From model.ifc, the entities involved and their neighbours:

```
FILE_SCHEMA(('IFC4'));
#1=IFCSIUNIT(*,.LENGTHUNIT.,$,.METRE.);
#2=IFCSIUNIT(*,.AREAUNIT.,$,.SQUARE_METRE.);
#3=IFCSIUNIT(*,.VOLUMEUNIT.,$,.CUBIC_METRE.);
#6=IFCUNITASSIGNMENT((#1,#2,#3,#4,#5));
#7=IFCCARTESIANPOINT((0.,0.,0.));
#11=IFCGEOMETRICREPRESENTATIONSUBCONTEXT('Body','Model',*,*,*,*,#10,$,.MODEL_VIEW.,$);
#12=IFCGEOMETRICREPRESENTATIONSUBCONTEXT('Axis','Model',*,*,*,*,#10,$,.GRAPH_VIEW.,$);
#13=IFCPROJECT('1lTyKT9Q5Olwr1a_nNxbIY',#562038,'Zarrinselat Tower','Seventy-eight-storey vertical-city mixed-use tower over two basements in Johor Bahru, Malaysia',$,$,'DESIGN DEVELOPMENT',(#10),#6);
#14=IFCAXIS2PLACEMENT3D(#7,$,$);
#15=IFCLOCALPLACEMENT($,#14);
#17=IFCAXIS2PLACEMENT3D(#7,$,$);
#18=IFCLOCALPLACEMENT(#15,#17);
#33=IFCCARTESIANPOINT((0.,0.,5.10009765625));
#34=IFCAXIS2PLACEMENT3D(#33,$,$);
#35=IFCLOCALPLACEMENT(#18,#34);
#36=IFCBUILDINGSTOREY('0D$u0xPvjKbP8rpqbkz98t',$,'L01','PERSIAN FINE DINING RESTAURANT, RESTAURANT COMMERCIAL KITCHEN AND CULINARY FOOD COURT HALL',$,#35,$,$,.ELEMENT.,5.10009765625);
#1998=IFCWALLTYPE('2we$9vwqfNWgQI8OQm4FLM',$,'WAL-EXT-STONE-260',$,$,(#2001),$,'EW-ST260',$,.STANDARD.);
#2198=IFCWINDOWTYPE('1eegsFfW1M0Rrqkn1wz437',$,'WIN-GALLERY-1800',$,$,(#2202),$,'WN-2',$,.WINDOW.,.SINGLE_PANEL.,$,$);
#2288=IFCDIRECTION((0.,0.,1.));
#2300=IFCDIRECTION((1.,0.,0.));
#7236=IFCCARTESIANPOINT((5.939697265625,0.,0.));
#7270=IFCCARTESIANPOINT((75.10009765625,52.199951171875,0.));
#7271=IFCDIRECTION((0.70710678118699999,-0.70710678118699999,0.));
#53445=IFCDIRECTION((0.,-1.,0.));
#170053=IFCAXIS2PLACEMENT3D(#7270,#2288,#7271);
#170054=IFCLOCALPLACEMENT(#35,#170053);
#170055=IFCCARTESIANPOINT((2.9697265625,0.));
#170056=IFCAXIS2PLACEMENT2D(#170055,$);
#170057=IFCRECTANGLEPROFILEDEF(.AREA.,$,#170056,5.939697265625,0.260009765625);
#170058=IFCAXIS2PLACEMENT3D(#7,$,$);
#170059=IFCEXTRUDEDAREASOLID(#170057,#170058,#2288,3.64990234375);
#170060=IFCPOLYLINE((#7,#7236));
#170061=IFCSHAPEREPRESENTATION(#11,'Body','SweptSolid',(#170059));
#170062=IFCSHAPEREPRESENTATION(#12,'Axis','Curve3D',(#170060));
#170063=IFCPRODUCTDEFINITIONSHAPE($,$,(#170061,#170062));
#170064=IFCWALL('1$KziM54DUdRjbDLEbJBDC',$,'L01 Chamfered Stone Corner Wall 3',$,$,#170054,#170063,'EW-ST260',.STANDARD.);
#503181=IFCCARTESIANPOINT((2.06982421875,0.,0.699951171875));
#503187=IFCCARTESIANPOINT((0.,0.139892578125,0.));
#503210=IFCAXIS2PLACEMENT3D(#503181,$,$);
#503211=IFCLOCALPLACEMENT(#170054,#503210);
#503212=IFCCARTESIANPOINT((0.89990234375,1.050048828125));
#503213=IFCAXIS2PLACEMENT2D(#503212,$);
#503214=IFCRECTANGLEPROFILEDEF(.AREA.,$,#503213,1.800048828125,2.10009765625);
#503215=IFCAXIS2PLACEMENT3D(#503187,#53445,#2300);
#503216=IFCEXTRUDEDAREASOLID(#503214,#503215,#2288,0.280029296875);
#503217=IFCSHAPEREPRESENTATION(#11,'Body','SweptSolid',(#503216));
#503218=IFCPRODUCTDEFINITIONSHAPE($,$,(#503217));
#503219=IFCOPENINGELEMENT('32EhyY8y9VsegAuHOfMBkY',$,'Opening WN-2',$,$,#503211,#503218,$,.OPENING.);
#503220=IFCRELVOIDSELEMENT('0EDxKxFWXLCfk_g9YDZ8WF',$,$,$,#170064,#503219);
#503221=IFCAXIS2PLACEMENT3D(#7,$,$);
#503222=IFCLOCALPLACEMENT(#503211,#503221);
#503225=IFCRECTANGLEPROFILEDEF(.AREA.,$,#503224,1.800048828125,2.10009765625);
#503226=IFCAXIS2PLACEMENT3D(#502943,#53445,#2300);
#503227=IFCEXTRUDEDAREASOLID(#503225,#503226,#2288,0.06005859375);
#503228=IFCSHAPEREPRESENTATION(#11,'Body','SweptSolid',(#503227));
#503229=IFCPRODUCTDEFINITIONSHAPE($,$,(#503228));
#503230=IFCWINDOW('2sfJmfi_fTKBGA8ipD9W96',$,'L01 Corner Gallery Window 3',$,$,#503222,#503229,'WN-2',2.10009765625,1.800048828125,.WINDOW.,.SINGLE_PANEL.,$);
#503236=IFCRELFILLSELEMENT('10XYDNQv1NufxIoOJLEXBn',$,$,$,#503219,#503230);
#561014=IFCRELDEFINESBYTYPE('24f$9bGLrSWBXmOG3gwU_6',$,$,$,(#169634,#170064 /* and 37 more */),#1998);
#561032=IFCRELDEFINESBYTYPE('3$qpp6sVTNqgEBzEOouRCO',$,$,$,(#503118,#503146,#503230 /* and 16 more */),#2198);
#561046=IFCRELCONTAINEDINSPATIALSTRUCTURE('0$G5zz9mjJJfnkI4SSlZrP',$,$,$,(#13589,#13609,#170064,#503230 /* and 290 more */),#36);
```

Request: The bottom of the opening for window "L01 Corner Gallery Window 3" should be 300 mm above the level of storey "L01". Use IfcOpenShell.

```python
import numpy as np
import ifcopenshell
import ifcopenshell.api.geometry
import ifcopenshell.geom
import ifcopenshell.util.element
import ifcopenshell.util.placement
import ifcopenshell.util.shape
import ifcopenshell.util.unit

model = ifcopenshell.open("model.ifc")
unit_scale = ifcopenshell.util.unit.calculate_unit_scale(model)

window = model.by_guid("2sfJmfi_fTKBGA8ipD9W96")
opening = window.FillsVoids[0].RelatingOpeningElement
storey = ifcopenshell.util.element.get_container(window, ifc_class="IfcBuildingStorey")
level = ifcopenshell.util.placement.get_local_placement(storey.ObjectPlacement)[2, 3]

# The opening's origin need not be at the sill, so measure its lowest point.
shape = ifcopenshell.geom.create_shape(ifcopenshell.geom.settings(), opening)
bottom = ifcopenshell.util.shape.get_shape_bottom_elevation(shape, shape.geometry) / unit_scale
dz = level + 0.3 - bottom

shift = np.array([0.0, 0.0, dz])
# The window is placed relative to its opening, so it follows when the opening moves.
matrix = ifcopenshell.util.placement.get_local_placement(opening.ObjectPlacement)
matrix[:3, 3] += shift
ifcopenshell.api.geometry.edit_object_placement(
    model, product=opening, matrix=matrix, is_si=False, should_transform_children=True
)

print(f"moved by {dz * unit_scale:+.3f} m")

model.write("model_rev.ifc")
```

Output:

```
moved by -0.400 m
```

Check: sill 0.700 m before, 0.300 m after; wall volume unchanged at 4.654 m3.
